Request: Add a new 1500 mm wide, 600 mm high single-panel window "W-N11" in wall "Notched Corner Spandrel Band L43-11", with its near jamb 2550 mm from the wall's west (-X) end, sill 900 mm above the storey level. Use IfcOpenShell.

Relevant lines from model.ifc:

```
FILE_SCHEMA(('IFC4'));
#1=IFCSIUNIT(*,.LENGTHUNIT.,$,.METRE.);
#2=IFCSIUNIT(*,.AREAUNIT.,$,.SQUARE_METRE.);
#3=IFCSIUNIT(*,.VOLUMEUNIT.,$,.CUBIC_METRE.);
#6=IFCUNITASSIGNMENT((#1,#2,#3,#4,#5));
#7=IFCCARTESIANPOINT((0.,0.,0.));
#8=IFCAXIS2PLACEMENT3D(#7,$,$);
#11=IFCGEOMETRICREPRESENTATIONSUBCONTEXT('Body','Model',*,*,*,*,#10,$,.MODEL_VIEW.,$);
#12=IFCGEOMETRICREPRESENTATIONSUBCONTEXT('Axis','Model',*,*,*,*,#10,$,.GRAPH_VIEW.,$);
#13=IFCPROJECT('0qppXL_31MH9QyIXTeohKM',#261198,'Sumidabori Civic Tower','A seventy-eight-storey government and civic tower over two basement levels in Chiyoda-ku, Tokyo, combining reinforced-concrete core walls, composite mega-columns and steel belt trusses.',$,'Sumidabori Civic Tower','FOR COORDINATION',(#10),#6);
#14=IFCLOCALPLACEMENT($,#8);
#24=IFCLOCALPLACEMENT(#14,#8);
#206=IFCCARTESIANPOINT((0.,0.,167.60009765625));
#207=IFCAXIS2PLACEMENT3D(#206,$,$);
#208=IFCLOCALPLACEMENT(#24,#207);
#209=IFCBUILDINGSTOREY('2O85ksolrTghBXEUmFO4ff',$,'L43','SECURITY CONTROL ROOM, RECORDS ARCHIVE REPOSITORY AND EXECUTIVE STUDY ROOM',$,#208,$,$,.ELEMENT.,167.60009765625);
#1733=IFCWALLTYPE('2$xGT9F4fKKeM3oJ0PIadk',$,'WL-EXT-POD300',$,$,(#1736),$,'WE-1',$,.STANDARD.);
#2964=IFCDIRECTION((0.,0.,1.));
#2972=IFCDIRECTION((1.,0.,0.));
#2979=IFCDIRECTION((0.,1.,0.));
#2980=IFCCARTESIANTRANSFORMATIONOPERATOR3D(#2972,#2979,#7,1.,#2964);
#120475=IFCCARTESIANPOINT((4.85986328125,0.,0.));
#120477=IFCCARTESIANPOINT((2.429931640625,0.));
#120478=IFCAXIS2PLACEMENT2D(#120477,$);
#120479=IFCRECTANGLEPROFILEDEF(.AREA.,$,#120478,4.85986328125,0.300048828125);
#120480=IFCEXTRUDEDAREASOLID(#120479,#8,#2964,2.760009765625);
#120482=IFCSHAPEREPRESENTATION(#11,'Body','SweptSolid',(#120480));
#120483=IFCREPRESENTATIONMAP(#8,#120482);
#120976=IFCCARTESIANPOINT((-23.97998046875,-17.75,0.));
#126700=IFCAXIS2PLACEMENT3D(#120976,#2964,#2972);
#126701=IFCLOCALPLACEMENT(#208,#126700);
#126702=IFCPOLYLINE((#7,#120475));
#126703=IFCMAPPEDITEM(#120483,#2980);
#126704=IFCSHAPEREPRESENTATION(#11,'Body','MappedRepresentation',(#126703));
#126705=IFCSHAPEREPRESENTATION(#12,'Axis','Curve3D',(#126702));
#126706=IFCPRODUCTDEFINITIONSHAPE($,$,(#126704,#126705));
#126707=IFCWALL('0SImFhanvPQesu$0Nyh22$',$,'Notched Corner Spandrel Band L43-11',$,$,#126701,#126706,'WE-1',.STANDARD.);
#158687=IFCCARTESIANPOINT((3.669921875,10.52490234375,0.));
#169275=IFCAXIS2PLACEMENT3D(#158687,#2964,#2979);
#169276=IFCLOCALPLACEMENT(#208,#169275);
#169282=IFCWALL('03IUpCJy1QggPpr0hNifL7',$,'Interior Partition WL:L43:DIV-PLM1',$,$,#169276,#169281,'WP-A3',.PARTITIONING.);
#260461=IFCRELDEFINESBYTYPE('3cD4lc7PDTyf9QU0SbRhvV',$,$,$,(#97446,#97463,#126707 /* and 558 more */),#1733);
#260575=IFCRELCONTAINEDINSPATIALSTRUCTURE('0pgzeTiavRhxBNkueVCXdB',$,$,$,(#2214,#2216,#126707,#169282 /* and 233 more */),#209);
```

```python
import numpy as np
import ifcopenshell
import ifcopenshell.api.feature
import ifcopenshell.api.geometry
import ifcopenshell.api.root
import ifcopenshell.api.spatial
import ifcopenshell.geom
import ifcopenshell.util.element
import ifcopenshell.util.placement
import ifcopenshell.util.representation
import ifcopenshell.util.shape
import ifcopenshell.util.unit

model = ifcopenshell.open("model.ifc")
unit_scale = ifcopenshell.util.unit.calculate_unit_scale(model)
settings = ifcopenshell.geom.settings()


def volume(element):
    """Net volume in cubic metres, openings subtracted."""
    shape = ifcopenshell.geom.create_shape(settings, element)
    return ifcopenshell.util.shape.get_volume(shape.geometry)


wall = model.by_guid("0SImFhanvPQesu$0Nyh22$")
storey = ifcopenshell.util.element.get_container(wall, ifc_class="IfcBuildingStorey")
context = ifcopenshell.util.representation.get_context(model, "Model", "Body", "MODEL_VIEW")
before = volume(wall)

width, height, from_end, sill = 1.5, 0.6, 2.55, 0.9  # metres

# The wall runs along its own X axis, and the end named is its -X end.
wall_shape = ifcopenshell.geom.create_shape(settings, wall)
x, y, z = ifcopenshell.util.shape.get_vertices(wall_shape.geometry).T
start = x.min() + from_end
face, thickness = float(y.min()), float(y.max() - y.min())
wall_matrix = ifcopenshell.util.placement.get_local_placement(wall.ObjectPlacement)
level = ifcopenshell.util.placement.get_local_placement(storey.ObjectPlacement)[2, 3]


def in_wall(x, y):
    """Placement at x, y metres in the wall's axes, at sill height."""
    matrix = wall_matrix.copy()
    matrix[:, 3] = wall_matrix @ np.array([x / unit_scale, y / unit_scale, 0.0, 1.0])
    matrix[2, 3] = level + sill / unit_scale
    return matrix


# Opening: a box that overshoots both wall faces by 50 mm.
opening = ifcopenshell.api.root.create_entity(model, ifc_class="IfcOpeningElement", predefined_type="OPENING")
box = ifcopenshell.api.geometry.add_wall_representation(
    model, context=context, length=width, height=height, thickness=thickness + 0.1
)
ifcopenshell.api.geometry.assign_representation(model, product=opening, representation=box)
ifcopenshell.api.geometry.edit_object_placement(model, product=opening, matrix=in_wall(start, face - 0.05), is_si=False)
ifcopenshell.api.feature.add_feature(model, feature=opening, element=wall)

window = ifcopenshell.api.root.create_entity(model, ifc_class="IfcWindow", name="W-N11", predefined_type="WINDOW")
window.OverallWidth, window.OverallHeight = width / unit_scale, height / unit_scale
window.PartitioningType = "SINGLE_PANEL"
body = ifcopenshell.api.geometry.add_window_representation(
    model,
    context=context,
    overall_width=window.OverallWidth,
    overall_height=window.OverallHeight,
    partition_type="SINGLE_PANEL",
)
ifcopenshell.api.geometry.assign_representation(model, product=window, representation=body)
ifcopenshell.api.spatial.assign_container(model, products=[window], relating_structure=storey)
ifcopenshell.api.feature.add_filling(model, opening=opening, element=window)

# Centre the window in the wall's thickness.
ifcopenshell.api.geometry.edit_object_placement(model, product=window, matrix=in_wall(start, face), is_si=False)
window_shape = ifcopenshell.geom.create_shape(settings, window)
depth = ifcopenshell.util.shape.get_vertices(window_shape.geometry)[:, 1]
offset = face + thickness / 2 - (depth.min() + depth.max()) / 2
ifcopenshell.api.geometry.edit_object_placement(model, product=window, matrix=in_wall(start, offset), is_si=False)

after = volume(wall)

print(f"wall volume {before:.3f} -> {after:.3f} m3")

model.write("model-out.ifc")
```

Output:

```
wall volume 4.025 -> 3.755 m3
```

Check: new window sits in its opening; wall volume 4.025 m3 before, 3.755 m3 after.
